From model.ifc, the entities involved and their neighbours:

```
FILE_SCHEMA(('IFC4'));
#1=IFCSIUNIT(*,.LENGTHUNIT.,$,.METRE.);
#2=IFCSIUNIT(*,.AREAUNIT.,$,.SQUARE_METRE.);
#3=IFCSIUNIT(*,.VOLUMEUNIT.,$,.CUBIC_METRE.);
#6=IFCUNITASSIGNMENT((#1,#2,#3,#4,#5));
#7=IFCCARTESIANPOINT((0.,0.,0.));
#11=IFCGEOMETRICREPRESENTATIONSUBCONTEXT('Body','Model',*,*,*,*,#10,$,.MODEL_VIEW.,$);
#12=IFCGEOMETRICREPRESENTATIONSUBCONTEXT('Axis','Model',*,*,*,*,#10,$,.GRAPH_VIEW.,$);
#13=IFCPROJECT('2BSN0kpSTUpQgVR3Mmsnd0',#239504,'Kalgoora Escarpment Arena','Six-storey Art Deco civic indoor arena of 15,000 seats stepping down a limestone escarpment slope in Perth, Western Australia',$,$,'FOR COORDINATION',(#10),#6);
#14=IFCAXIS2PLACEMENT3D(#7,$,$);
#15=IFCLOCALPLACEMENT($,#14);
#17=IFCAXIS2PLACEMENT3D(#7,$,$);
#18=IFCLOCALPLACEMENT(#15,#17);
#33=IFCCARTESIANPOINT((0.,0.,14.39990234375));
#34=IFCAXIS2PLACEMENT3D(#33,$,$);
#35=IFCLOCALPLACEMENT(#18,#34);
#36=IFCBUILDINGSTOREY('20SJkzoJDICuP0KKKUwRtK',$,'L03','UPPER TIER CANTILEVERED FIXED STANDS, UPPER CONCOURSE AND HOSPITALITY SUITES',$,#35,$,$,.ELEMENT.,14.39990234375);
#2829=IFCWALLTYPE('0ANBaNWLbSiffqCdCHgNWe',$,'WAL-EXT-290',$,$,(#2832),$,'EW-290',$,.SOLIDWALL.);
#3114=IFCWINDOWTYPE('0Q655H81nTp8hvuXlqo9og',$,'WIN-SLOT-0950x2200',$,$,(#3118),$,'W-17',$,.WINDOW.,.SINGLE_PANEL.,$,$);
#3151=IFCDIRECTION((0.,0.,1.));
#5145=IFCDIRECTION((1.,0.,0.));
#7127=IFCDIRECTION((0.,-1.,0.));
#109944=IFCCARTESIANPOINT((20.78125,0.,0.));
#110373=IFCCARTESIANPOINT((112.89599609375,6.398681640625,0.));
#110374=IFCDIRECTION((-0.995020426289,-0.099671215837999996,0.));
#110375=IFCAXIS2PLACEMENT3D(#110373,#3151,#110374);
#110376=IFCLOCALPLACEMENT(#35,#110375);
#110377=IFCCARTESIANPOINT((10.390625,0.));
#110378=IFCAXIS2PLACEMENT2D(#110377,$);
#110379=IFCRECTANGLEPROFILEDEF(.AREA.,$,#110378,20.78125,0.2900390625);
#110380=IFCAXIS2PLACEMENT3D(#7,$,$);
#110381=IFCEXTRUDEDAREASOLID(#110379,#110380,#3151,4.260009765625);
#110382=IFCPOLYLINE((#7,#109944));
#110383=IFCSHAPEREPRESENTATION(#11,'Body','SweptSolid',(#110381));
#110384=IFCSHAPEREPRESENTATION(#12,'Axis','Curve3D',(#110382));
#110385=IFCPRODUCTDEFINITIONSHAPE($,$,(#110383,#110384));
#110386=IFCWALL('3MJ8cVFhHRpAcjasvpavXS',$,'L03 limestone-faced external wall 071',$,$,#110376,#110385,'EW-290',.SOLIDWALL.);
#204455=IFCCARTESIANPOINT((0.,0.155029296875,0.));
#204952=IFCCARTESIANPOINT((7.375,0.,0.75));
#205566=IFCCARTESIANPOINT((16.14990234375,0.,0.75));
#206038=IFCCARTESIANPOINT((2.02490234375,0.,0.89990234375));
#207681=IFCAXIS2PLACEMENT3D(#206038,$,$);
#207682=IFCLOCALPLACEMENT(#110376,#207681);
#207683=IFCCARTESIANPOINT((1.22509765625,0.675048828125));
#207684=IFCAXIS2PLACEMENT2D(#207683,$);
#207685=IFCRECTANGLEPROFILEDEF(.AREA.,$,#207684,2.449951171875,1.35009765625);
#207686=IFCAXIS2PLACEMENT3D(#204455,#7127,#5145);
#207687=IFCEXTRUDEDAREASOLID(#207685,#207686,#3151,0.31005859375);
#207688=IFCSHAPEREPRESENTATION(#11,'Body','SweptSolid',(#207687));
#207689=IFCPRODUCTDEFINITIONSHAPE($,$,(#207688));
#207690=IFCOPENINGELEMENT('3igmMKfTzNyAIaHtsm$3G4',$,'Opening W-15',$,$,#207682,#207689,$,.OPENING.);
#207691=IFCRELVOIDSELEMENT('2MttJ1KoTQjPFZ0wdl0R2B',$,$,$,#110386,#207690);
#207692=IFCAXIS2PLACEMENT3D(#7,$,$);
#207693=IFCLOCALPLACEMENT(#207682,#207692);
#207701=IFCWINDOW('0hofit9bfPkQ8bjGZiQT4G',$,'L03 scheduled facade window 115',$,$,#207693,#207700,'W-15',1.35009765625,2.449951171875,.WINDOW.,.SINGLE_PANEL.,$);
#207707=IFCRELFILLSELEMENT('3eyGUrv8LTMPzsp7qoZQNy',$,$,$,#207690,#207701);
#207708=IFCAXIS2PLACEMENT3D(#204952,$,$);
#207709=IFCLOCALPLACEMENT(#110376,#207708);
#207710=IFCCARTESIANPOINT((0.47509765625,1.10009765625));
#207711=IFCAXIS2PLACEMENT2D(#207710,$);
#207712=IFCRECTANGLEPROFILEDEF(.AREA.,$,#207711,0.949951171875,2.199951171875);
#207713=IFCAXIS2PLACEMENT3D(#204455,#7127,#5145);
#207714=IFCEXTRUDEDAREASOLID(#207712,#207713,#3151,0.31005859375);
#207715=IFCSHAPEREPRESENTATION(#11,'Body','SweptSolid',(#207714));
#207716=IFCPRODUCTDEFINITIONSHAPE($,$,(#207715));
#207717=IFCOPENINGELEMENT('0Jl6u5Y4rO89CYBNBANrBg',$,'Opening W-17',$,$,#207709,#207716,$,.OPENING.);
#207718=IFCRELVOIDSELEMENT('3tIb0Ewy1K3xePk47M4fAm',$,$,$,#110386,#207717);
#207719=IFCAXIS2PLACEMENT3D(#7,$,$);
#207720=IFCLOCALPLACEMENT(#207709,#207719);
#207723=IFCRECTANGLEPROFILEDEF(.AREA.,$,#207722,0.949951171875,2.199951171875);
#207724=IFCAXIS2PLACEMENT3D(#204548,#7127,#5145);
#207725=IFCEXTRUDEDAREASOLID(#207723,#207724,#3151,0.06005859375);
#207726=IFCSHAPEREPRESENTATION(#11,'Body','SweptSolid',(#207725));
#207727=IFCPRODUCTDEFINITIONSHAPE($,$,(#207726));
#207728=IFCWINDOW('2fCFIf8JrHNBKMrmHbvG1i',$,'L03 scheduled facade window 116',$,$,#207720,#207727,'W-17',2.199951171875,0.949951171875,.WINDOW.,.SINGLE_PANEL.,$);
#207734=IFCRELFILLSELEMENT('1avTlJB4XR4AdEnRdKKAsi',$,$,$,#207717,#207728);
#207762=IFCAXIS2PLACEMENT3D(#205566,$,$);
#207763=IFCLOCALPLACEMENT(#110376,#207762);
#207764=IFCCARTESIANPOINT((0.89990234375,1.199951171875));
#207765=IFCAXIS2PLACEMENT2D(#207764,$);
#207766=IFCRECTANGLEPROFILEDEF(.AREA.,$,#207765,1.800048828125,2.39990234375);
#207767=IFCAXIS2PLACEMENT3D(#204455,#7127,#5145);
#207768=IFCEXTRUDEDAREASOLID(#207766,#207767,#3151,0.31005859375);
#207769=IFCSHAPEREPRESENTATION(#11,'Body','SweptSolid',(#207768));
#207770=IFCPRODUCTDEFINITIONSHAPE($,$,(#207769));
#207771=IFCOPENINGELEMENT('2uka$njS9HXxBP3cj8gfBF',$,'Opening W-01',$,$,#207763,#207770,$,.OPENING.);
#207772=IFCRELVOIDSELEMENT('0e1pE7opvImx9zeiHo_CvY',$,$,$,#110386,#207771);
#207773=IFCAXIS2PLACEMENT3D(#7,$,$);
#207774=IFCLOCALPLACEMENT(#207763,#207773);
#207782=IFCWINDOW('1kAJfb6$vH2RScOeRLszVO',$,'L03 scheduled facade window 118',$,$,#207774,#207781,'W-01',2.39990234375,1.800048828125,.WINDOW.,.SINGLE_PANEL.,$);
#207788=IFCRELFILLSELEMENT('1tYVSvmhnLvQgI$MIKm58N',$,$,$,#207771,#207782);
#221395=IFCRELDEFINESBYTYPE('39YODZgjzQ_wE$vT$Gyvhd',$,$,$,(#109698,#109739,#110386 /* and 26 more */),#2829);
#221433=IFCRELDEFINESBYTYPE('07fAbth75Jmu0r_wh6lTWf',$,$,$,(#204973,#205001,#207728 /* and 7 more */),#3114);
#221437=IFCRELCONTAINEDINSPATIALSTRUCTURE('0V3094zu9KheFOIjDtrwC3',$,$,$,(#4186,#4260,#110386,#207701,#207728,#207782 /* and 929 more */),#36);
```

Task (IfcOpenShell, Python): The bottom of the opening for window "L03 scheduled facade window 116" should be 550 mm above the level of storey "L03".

```python
import numpy as np
import ifcopenshell
import ifcopenshell.api.geometry
import ifcopenshell.geom
import ifcopenshell.util.element
import ifcopenshell.util.placement
import ifcopenshell.util.shape
import ifcopenshell.util.unit

model = ifcopenshell.open("model.ifc")
unit_scale = ifcopenshell.util.unit.calculate_unit_scale(model)

window = model.by_guid("2fCFIf8JrHNBKMrmHbvG1i")
opening = window.FillsVoids[0].RelatingOpeningElement
storey = ifcopenshell.util.element.get_container(window, ifc_class="IfcBuildingStorey")
level = ifcopenshell.util.placement.get_local_placement(storey.ObjectPlacement)[2, 3]

# The opening's origin need not be at the sill, so measure its lowest point.
shape = ifcopenshell.geom.create_shape(ifcopenshell.geom.settings(), opening)
bottom = ifcopenshell.util.shape.get_shape_bottom_elevation(shape, shape.geometry) / unit_scale
dz = level + 0.55 - bottom

shift = np.array([0.0, 0.0, dz])
# The window is placed relative to its opening, so it follows when the opening moves.
matrix = ifcopenshell.util.placement.get_local_placement(opening.ObjectPlacement)
matrix[:3, 3] += shift
ifcopenshell.api.geometry.edit_object_placement(
    model, product=opening, matrix=matrix, is_si=False, should_transform_children=True
)

print(f"moved by {dz * unit_scale:+.3f} m")

model.write("model_rev.ifc")
```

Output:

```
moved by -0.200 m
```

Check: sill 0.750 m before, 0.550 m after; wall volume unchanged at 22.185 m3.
